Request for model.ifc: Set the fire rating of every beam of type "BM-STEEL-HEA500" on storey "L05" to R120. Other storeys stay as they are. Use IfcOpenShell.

First a look at what the model holds.

```python
import ifcopenshell
import ifcopenshell.util.element

model = ifcopenshell.open("model.ifc")
print(model.schema)
storey = next(s for s in model.by_type("IfcBuildingStorey") if s.Name == "L05")
beams = [e for e in ifcopenshell.util.element.get_decomposition(storey) if e.is_a("IfcBeam")]
seen = {}
for e in beams:
    element_type = ifcopenshell.util.element.get_type(e)
    key = (element_type.Name if element_type != e and element_type else None, ifcopenshell.util.element.get_pset(e, "Pset_BeamCommon", "FireRating"))
    seen[key] = seen.get(key, 0) + 1
for (name, value), count in sorted(seen.items(), key=str):
    print(count, "x", name, "|", value)
```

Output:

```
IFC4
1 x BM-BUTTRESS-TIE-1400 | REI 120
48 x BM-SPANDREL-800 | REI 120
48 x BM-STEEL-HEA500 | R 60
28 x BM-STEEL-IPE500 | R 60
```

```python
import ifcopenshell
import ifcopenshell.api.pset
import ifcopenshell.util.element

model = ifcopenshell.open("model.ifc")

storey = next(s for s in model.by_type("IfcBuildingStorey") if s.Name == "L05")
beams = [e for e in ifcopenshell.util.element.get_decomposition(storey) if e.is_a("IfcBeam")]

count = 0
for e in beams:
    element_type = ifcopenshell.util.element.get_type(e)
    if element_type in (None, e) or element_type.Name != "BM-STEEL-HEA500":
        continue
    # add_pset returns the element's existing set when there is one.
    pset = ifcopenshell.api.pset.add_pset(model, product=e, name="Pset_BeamCommon")
    ifcopenshell.api.pset.edit_pset(model, pset=pset, properties={"FireRating": "R120"})
    count += 1

print(count, "beams updated")

model.write("model_rev.ifc")
```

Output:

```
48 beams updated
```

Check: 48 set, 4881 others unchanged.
